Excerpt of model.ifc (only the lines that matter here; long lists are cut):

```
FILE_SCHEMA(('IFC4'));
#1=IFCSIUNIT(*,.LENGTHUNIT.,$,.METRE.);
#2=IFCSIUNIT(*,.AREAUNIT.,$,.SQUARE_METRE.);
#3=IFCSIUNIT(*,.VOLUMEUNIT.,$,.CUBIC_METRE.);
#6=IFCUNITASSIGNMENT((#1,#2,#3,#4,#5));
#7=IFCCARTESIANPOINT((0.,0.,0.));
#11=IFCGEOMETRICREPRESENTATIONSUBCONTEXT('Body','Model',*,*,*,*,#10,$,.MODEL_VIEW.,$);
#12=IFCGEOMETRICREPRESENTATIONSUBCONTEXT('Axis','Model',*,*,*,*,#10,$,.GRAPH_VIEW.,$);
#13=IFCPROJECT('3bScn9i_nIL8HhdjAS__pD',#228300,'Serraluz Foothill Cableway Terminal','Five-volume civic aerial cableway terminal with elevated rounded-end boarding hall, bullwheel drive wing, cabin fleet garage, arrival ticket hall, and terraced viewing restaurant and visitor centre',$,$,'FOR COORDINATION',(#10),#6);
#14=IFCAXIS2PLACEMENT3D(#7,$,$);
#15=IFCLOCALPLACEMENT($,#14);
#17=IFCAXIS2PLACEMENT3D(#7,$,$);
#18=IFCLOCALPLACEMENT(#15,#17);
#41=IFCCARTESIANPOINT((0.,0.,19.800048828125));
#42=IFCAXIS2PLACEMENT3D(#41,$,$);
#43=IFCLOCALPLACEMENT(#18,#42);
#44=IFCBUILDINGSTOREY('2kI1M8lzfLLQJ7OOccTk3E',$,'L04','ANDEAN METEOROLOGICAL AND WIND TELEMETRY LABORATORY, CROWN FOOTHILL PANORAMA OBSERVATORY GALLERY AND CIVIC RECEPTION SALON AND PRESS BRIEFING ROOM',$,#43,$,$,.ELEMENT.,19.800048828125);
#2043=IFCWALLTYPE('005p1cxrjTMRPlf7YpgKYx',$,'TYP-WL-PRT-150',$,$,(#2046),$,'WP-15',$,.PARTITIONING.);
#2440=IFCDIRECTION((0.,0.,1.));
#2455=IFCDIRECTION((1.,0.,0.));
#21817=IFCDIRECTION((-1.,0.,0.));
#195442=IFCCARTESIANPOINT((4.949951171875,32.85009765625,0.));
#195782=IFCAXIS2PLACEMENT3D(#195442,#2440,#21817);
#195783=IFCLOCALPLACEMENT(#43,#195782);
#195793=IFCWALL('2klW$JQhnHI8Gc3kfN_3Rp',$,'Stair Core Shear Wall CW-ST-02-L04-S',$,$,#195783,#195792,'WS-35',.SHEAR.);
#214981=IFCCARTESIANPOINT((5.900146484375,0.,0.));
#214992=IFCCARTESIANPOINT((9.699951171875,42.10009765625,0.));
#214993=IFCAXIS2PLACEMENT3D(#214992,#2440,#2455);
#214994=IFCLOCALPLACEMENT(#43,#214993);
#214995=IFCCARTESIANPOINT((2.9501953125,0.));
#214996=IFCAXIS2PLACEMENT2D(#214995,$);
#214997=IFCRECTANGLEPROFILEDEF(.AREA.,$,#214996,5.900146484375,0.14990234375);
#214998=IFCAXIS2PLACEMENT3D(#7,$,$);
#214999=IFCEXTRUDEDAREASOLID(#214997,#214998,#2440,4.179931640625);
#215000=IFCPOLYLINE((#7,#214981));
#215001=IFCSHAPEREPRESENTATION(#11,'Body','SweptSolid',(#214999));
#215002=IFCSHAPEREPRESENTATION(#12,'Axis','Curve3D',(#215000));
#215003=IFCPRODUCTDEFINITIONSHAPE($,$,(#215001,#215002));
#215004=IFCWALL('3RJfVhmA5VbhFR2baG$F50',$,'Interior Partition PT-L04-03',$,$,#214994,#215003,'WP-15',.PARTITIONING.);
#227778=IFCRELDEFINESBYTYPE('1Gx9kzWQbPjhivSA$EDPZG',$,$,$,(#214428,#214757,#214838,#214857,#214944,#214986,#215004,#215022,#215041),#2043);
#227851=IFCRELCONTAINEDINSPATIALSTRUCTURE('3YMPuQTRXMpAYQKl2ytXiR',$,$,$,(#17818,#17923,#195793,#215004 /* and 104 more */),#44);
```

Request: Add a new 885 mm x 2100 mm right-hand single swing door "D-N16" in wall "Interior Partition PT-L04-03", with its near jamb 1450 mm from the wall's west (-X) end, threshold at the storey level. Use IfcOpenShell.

```python
import numpy as np
import ifcopenshell
import ifcopenshell.api.feature
import ifcopenshell.api.geometry
import ifcopenshell.api.root
import ifcopenshell.api.spatial
import ifcopenshell.geom
import ifcopenshell.util.element
import ifcopenshell.util.placement
import ifcopenshell.util.representation
import ifcopenshell.util.shape
import ifcopenshell.util.unit

model = ifcopenshell.open("model.ifc")
unit_scale = ifcopenshell.util.unit.calculate_unit_scale(model)
settings = ifcopenshell.geom.settings()


def volume(element):
    """Net volume in cubic metres, openings subtracted."""
    shape = ifcopenshell.geom.create_shape(settings, element)
    return ifcopenshell.util.shape.get_volume(shape.geometry)


wall = model.by_guid("3RJfVhmA5VbhFR2baG$F50")
storey = ifcopenshell.util.element.get_container(wall, ifc_class="IfcBuildingStorey")
context = ifcopenshell.util.representation.get_context(model, "Model", "Body", "MODEL_VIEW")
before = volume(wall)

width, height, from_end, sill = 0.885, 2.1, 1.45, 0.0  # metres

# The wall runs along its own X axis, and the end named is its -X end.
wall_shape = ifcopenshell.geom.create_shape(settings, wall)
x, y, z = ifcopenshell.util.shape.get_vertices(wall_shape.geometry).T
start = x.min() + from_end
face, thickness = float(y.min()), float(y.max() - y.min())
wall_matrix = ifcopenshell.util.placement.get_local_placement(wall.ObjectPlacement)
level = ifcopenshell.util.placement.get_local_placement(storey.ObjectPlacement)[2, 3]


def in_wall(x, y):
    """Placement at x, y metres in the wall's axes, at sill height."""
    matrix = wall_matrix.copy()
    matrix[:, 3] = wall_matrix @ np.array([x / unit_scale, y / unit_scale, 0.0, 1.0])
    matrix[2, 3] = level + sill / unit_scale
    return matrix


# Opening: a box that overshoots both wall faces by 50 mm.
opening = ifcopenshell.api.root.create_entity(model, ifc_class="IfcOpeningElement", predefined_type="OPENING")
box = ifcopenshell.api.geometry.add_wall_representation(
    model, context=context, length=width, height=height, thickness=thickness + 0.1
)
ifcopenshell.api.geometry.assign_representation(model, product=opening, representation=box)
ifcopenshell.api.geometry.edit_object_placement(model, product=opening, matrix=in_wall(start, face - 0.05), is_si=False)
ifcopenshell.api.feature.add_feature(model, feature=opening, element=wall)

door = ifcopenshell.api.root.create_entity(model, ifc_class="IfcDoor", name="D-N16", predefined_type="DOOR")
door.OverallWidth, door.OverallHeight = width / unit_scale, height / unit_scale
door.OperationType = "SINGLE_SWING_RIGHT"
body = ifcopenshell.api.geometry.add_door_representation(
    model,
    context=context,
    overall_width=door.OverallWidth,
    overall_height=door.OverallHeight,
    operation_type="SINGLE_SWING_RIGHT",
    lining_properties={"LiningDepth": thickness / unit_scale, "ThresholdDepth": thickness / unit_scale},
)
ifcopenshell.api.geometry.assign_representation(model, product=door, representation=body)
ifcopenshell.api.spatial.assign_container(model, products=[door], relating_structure=storey)
ifcopenshell.api.feature.add_filling(model, opening=opening, element=door)

# The lining spans the wall, so the door starts at the wall face.
ifcopenshell.api.geometry.edit_object_placement(model, product=door, matrix=in_wall(start, face), is_si=False)

after = volume(wall)

print(f"wall volume {before:.3f} -> {after:.3f} m3")

model.write("model_v2.ifc")
```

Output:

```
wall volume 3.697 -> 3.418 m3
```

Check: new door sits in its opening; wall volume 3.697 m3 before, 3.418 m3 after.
